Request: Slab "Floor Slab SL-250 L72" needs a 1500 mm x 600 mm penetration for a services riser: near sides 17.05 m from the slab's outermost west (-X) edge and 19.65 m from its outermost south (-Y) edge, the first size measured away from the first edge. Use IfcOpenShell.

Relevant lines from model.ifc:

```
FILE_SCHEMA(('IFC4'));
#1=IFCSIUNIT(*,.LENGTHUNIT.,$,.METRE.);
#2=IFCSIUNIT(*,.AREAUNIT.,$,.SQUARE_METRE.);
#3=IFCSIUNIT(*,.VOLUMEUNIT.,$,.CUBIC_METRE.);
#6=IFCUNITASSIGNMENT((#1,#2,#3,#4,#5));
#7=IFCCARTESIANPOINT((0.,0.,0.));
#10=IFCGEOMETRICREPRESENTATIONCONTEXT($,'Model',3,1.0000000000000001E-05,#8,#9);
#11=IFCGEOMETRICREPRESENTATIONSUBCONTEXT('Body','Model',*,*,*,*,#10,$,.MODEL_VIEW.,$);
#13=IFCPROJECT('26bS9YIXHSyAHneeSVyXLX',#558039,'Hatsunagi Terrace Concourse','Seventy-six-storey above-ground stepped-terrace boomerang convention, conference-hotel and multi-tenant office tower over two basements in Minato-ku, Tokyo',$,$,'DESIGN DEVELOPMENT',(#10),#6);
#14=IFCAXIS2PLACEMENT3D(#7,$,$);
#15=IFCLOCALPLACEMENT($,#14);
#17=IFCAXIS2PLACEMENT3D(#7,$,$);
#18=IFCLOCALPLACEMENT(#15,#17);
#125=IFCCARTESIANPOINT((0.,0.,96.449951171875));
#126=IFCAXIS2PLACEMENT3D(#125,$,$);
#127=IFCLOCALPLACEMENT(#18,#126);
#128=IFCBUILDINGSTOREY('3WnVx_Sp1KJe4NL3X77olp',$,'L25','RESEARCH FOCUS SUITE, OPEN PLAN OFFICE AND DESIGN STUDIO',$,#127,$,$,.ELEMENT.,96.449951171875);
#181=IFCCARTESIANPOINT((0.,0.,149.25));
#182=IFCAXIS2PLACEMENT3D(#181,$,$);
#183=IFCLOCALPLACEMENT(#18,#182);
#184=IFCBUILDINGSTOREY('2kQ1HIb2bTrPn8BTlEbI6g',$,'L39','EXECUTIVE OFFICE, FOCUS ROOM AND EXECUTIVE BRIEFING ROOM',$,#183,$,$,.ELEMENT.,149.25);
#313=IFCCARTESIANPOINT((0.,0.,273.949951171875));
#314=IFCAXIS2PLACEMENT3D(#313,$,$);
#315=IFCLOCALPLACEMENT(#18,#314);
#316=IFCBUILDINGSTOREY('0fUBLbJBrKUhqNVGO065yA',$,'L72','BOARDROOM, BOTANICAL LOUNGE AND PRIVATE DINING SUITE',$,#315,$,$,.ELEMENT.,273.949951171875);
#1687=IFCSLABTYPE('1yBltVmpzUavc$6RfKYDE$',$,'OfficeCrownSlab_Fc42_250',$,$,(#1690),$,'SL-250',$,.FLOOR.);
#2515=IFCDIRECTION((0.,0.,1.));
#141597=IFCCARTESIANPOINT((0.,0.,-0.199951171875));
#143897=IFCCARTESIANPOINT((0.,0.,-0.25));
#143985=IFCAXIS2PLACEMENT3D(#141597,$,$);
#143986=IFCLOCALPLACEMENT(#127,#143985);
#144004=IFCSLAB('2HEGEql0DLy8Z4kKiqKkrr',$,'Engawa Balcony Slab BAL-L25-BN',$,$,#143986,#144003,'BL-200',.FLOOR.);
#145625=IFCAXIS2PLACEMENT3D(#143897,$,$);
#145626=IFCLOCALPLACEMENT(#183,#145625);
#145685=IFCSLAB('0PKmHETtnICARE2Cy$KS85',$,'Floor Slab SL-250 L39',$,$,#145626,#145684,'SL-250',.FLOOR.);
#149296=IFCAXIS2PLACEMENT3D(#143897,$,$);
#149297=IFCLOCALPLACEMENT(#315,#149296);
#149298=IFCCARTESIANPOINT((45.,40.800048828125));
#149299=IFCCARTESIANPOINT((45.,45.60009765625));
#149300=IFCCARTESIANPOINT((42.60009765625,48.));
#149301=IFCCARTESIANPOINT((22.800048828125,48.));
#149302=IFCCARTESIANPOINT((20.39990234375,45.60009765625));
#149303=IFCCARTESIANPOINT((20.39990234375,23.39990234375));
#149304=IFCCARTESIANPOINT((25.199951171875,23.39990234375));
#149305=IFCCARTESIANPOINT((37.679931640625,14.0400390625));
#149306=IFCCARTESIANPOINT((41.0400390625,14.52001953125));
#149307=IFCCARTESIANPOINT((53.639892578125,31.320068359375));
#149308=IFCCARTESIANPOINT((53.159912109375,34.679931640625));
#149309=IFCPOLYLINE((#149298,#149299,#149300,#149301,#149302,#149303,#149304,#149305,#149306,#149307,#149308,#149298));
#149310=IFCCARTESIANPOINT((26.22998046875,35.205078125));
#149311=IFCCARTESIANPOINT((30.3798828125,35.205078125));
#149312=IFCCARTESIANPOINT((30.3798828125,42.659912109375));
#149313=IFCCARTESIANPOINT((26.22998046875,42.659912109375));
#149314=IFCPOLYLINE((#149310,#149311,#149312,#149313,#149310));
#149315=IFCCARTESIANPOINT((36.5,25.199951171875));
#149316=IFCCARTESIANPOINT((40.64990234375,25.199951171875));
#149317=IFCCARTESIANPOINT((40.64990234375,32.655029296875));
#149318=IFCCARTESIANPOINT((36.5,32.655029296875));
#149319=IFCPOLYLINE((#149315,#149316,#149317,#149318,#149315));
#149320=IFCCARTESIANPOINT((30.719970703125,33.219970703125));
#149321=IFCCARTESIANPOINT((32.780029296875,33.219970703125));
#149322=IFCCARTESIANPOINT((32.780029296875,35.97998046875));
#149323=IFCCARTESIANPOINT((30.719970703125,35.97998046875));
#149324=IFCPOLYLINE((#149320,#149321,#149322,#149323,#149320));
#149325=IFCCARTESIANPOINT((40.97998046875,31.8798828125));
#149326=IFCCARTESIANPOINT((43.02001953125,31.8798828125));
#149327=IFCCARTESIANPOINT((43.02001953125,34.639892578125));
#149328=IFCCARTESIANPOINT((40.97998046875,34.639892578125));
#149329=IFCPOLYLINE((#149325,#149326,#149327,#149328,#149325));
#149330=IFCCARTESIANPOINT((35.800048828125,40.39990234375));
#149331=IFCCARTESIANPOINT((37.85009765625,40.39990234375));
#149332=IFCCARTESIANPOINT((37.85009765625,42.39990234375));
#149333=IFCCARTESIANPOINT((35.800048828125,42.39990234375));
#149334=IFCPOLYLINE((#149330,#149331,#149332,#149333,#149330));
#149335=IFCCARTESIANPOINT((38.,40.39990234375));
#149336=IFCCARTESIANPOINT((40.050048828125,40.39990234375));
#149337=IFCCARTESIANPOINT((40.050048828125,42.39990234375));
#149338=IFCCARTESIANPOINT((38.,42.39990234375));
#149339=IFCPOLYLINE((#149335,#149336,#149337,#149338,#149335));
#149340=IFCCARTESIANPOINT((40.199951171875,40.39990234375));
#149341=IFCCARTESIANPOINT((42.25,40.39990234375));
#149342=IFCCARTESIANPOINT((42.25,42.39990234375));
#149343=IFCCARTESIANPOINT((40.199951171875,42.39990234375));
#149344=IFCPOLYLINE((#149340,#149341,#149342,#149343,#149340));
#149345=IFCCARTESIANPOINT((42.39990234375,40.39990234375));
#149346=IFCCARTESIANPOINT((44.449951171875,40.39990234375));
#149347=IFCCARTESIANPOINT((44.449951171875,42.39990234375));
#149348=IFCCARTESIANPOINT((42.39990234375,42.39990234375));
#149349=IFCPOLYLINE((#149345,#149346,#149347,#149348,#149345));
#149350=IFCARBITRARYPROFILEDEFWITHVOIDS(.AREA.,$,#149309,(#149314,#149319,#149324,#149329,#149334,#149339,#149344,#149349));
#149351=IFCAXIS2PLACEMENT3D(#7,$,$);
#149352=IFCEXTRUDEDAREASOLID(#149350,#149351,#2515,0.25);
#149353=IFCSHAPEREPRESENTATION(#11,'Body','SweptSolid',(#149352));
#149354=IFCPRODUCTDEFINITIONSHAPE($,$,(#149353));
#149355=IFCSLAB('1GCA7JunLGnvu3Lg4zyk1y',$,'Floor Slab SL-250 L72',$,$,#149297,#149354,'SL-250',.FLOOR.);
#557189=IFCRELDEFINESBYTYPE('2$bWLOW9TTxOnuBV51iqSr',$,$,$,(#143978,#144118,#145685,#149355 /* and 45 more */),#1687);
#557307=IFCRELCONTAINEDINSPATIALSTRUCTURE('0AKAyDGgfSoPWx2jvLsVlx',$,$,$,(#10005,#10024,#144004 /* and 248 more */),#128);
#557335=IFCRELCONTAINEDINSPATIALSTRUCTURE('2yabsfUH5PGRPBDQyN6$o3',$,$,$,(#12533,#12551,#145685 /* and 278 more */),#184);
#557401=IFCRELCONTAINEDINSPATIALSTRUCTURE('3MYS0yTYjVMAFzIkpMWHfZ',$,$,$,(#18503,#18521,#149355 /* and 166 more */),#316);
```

```python
import numpy as np
import ifcopenshell
import ifcopenshell.api.feature
import ifcopenshell.api.geometry
import ifcopenshell.api.root
import ifcopenshell.geom
import ifcopenshell.util.placement
import ifcopenshell.util.representation
import ifcopenshell.util.shape
import ifcopenshell.util.unit

model = ifcopenshell.open("model.ifc")
unit_scale = ifcopenshell.util.unit.calculate_unit_scale(model)
settings = ifcopenshell.geom.settings()


def volume(element):
    """Net volume in cubic metres, openings subtracted."""
    shape = ifcopenshell.geom.create_shape(settings, element)
    return ifcopenshell.util.shape.get_volume(shape.geometry)


slab = model.by_id(149355)
before = volume(slab)

# Extent in the slab's own axes, in metres. The edges named are its -X and -Y sides.
slab_shape = ifcopenshell.geom.create_shape(settings, slab)
vertices = ifcopenshell.util.shape.get_vertices(slab_shape.geometry)
x_min, y_min, bottom = vertices.min(axis=0)
top = vertices[:, 2].max()

opening = ifcopenshell.api.root.create_entity(model, ifc_class="IfcOpeningElement", name="Services riser opening", predefined_type="OPENING")
context = ifcopenshell.util.representation.get_context(model, "Model", "Body", "MODEL_VIEW")
width, depth = 1.5, 0.6
outline = [(0.0, 0.0), (width, 0.0), (width, depth), (0.0, depth), (0.0, 0.0)]
# Overshoot both faces by 50 mm so the cut is clean.
shape = ifcopenshell.api.geometry.add_slab_representation(
    model, context=context, depth=top - bottom + 0.1, polyline=outline
)
ifcopenshell.api.geometry.assign_representation(model, product=opening, representation=shape)

matrix = ifcopenshell.util.placement.get_local_placement(slab.ObjectPlacement)
matrix[:, 3] = matrix @ np.append(np.array([x_min + 17.05, y_min + 19.65, bottom - 0.05]) / unit_scale, 1.0)
ifcopenshell.api.geometry.edit_object_placement(model, product=opening, matrix=matrix, is_si=False)
ifcopenshell.api.feature.add_feature(model, feature=opening, element=slab)

after = volume(slab)

print(f"slab volume {before:.3f} -> {after:.3f} m3")

model.write("model-out.ifc")
```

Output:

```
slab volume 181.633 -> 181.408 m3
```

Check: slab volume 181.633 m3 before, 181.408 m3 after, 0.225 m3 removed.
